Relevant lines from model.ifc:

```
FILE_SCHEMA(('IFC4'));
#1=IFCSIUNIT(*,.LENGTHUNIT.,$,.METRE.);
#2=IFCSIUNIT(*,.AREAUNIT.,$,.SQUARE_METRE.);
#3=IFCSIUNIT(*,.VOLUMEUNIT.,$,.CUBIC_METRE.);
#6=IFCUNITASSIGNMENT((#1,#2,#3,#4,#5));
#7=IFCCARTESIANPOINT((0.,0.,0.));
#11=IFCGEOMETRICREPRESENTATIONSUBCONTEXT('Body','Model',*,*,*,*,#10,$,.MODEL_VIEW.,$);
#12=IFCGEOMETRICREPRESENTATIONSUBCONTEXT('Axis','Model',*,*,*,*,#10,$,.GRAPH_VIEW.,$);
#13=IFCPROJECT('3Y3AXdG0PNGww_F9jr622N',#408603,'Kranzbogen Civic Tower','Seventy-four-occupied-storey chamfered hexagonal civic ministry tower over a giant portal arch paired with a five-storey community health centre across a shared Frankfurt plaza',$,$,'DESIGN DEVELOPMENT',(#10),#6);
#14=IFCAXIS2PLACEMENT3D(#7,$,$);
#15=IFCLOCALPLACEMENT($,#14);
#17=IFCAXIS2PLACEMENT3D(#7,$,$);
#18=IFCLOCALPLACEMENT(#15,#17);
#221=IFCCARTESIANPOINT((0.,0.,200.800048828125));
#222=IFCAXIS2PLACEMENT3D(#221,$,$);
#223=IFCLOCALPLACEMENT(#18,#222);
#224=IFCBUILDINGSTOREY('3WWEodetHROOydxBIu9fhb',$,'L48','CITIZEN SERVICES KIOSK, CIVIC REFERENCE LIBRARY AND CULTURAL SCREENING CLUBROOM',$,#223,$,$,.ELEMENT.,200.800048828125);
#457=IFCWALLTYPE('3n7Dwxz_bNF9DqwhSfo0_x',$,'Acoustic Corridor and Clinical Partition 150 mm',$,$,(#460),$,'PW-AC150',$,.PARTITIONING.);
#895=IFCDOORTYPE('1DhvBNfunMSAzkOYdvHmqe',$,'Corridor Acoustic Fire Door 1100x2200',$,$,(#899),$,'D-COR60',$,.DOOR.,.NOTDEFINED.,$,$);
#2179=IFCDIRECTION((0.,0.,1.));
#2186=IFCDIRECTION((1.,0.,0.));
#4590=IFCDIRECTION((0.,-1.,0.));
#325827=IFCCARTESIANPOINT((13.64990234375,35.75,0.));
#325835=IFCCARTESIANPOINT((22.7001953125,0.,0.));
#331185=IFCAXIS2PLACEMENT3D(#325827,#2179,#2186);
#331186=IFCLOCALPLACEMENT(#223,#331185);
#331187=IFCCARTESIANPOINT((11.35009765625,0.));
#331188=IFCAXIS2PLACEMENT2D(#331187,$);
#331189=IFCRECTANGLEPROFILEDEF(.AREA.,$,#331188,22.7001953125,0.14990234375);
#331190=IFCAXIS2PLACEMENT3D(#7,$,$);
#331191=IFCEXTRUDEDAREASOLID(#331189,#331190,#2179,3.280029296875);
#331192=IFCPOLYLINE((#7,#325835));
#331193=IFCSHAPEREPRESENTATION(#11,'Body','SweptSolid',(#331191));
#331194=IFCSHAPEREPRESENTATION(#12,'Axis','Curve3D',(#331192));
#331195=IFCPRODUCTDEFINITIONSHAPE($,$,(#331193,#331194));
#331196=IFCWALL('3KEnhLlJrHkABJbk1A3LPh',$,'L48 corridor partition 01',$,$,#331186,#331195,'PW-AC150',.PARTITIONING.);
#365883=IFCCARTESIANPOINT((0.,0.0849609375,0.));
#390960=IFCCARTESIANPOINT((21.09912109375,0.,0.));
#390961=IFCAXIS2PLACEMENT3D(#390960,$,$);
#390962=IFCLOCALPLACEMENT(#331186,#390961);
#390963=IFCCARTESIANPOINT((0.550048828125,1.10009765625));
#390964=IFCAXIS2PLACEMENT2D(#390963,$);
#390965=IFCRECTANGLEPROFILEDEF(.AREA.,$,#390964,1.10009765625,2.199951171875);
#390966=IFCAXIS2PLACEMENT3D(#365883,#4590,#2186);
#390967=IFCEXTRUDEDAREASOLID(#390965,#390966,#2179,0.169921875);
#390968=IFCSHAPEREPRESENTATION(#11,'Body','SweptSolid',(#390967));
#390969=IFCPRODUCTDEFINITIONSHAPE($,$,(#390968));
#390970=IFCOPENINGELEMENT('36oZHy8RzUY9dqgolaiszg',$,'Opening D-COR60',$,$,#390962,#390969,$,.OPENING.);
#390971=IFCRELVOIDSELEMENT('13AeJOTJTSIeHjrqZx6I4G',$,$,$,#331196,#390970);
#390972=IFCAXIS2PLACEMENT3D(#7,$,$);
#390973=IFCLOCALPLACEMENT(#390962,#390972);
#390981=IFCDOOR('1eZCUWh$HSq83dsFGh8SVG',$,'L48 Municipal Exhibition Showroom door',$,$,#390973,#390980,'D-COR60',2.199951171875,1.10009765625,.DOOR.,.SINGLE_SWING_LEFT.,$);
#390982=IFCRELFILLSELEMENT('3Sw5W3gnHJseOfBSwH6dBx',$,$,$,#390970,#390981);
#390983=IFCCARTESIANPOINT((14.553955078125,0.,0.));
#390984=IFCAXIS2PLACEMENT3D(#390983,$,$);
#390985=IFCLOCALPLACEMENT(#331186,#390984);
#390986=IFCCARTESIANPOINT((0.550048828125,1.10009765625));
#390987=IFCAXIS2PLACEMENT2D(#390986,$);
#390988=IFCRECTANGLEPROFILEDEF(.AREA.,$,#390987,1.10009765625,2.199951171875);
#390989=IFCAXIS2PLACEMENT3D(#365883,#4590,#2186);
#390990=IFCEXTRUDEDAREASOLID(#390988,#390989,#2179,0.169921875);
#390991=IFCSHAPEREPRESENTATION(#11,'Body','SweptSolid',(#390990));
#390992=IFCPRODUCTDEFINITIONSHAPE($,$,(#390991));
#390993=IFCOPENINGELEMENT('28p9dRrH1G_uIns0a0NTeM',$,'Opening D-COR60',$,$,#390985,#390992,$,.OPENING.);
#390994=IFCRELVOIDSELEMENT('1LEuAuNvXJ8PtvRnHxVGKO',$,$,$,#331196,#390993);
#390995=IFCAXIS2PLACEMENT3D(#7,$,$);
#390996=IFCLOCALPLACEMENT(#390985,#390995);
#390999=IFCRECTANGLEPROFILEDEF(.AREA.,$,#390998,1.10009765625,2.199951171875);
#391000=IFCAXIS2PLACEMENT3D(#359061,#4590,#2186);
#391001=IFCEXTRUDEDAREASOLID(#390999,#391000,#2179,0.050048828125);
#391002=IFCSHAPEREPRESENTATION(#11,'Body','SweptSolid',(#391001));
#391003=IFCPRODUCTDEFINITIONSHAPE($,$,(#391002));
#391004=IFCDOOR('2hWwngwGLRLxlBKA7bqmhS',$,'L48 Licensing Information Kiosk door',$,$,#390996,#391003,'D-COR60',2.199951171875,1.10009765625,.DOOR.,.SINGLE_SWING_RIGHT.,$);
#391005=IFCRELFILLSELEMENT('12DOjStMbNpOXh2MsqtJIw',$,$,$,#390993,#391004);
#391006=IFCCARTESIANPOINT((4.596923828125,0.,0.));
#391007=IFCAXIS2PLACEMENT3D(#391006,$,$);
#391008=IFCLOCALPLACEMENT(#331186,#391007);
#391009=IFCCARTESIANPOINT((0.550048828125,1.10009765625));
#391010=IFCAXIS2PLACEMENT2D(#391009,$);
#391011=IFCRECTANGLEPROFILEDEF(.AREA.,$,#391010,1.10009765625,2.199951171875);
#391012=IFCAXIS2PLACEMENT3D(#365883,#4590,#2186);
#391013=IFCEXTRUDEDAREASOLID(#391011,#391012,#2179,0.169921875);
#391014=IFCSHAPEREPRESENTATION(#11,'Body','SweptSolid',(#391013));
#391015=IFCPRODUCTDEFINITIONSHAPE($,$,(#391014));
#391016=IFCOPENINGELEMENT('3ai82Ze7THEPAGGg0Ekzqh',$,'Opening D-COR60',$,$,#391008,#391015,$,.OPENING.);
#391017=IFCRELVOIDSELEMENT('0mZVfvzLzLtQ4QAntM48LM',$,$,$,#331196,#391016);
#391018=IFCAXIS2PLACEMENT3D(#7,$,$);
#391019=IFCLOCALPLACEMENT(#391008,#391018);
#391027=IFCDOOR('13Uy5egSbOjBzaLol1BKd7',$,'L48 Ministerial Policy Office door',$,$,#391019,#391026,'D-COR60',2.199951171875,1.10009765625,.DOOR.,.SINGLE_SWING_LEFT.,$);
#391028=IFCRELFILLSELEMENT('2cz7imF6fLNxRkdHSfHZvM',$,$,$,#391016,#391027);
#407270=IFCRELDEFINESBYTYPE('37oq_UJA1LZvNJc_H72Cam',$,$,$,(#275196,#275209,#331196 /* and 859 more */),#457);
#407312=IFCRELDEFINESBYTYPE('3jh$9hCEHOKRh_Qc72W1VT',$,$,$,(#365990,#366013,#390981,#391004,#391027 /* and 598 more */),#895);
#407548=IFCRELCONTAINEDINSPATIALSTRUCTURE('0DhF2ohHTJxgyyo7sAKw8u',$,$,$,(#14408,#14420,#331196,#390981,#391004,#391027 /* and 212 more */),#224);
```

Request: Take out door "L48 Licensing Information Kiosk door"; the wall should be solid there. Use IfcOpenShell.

```python
import ifcopenshell
import ifcopenshell.api.feature
import ifcopenshell.api.root
import ifcopenshell.geom
import ifcopenshell.util.shape

model = ifcopenshell.open("model.ifc")
settings = ifcopenshell.geom.settings()


def volume(element):
    """Net volume in cubic metres, openings subtracted."""
    shape = ifcopenshell.geom.create_shape(settings, element)
    return ifcopenshell.util.shape.get_volume(shape.geometry)


door = model.by_guid("2hWwngwGLRLxlBKA7bqmhS")
opening = door.FillsVoids[0].RelatingOpeningElement
wall = opening.VoidsElements[0].RelatingBuildingElement
before = volume(wall)

ifcopenshell.api.root.remove_product(model, product=door)
ifcopenshell.api.feature.remove_feature(model, feature=opening)

after = volume(wall)

print(f"wall volume {before:.3f} -> {after:.3f} m3")

model.write("model_updated.ifc")
```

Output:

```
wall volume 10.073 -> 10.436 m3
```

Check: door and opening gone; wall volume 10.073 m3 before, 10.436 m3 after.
